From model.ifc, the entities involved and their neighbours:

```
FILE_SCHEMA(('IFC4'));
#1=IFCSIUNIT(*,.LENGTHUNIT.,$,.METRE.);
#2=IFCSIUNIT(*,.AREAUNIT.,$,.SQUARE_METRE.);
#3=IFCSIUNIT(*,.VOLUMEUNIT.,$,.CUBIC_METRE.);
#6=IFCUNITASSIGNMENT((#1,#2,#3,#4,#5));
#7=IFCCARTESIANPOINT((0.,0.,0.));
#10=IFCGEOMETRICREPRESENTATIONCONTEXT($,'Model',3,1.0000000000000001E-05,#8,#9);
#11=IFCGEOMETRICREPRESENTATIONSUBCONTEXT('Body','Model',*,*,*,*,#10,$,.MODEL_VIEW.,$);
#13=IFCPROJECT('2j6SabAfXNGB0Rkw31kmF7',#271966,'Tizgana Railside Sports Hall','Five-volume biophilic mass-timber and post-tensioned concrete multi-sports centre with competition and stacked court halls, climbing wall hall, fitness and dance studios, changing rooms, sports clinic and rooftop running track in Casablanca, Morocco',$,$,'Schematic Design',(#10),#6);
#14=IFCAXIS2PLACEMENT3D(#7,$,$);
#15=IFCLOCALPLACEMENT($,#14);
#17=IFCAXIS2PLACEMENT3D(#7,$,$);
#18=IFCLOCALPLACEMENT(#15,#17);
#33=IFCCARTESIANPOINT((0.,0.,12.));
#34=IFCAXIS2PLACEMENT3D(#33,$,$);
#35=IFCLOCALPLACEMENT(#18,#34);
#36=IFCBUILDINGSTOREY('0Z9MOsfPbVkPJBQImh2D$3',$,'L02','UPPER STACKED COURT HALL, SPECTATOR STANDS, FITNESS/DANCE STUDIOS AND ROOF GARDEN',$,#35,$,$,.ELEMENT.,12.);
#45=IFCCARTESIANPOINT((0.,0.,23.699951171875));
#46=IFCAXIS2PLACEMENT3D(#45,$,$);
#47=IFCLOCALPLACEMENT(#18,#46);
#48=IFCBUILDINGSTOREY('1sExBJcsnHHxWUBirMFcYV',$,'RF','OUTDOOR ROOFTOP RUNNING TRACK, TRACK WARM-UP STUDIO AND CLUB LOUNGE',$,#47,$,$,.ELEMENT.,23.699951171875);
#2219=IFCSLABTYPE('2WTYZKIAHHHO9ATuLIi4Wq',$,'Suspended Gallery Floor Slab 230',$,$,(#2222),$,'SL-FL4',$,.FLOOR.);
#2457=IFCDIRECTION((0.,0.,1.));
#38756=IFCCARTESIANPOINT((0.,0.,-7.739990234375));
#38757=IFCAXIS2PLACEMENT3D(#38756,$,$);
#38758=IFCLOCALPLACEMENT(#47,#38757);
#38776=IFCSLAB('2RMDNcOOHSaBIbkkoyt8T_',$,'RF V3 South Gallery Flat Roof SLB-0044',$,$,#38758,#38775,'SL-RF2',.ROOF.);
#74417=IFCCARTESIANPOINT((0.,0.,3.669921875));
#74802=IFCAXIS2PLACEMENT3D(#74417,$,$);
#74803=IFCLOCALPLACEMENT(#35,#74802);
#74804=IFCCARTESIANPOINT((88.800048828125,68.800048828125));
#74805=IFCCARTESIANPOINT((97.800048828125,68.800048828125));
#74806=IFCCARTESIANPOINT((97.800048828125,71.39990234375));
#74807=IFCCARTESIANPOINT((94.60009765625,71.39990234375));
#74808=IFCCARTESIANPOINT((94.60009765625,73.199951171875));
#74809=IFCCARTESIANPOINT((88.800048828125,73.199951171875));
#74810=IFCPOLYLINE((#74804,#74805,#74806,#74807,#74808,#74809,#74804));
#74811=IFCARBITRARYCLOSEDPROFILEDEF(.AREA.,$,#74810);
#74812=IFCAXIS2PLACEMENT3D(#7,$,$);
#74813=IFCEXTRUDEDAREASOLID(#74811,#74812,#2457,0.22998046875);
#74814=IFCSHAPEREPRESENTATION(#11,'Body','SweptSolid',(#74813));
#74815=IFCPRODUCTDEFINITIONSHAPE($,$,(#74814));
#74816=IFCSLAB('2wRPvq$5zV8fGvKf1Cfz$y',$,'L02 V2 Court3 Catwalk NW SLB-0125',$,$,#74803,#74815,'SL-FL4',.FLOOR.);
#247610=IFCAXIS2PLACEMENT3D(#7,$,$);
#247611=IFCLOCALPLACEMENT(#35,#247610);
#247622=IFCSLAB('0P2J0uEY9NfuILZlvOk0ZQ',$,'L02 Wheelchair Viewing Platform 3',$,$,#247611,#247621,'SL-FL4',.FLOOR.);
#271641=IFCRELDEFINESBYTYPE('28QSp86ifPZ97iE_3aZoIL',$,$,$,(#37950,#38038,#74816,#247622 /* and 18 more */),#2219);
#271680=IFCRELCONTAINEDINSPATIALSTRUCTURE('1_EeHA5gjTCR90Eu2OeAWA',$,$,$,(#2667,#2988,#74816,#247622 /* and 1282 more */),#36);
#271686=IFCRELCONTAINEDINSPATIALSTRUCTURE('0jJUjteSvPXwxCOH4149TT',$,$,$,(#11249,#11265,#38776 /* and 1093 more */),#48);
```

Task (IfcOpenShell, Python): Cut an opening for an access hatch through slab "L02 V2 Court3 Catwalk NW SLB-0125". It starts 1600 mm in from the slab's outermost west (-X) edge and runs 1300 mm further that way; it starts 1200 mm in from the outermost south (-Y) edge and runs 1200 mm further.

```python
import numpy as np
import ifcopenshell
import ifcopenshell.api.feature
import ifcopenshell.api.geometry
import ifcopenshell.api.root
import ifcopenshell.geom
import ifcopenshell.util.placement
import ifcopenshell.util.representation
import ifcopenshell.util.shape
import ifcopenshell.util.unit

model = ifcopenshell.open("model.ifc")
unit_scale = ifcopenshell.util.unit.calculate_unit_scale(model)
settings = ifcopenshell.geom.settings()


def volume(element):
    """Net volume in cubic metres, openings subtracted."""
    shape = ifcopenshell.geom.create_shape(settings, element)
    return ifcopenshell.util.shape.get_volume(shape.geometry)


slab = model.by_id(74816)
before = volume(slab)

# Extent in the slab's own axes, in metres. The edges named are its -X and -Y sides.
slab_shape = ifcopenshell.geom.create_shape(settings, slab)
vertices = ifcopenshell.util.shape.get_vertices(slab_shape.geometry)
x_min, y_min, bottom = vertices.min(axis=0)
top = vertices[:, 2].max()

opening = ifcopenshell.api.root.create_entity(model, ifc_class="IfcOpeningElement", name="Access hatch opening", predefined_type="OPENING")
context = ifcopenshell.util.representation.get_context(model, "Model", "Body", "MODEL_VIEW")
width, depth = 1.3, 1.2
outline = [(0.0, 0.0), (width, 0.0), (width, depth), (0.0, depth), (0.0, 0.0)]
# Overshoot both faces by 50 mm so the cut is clean.
shape = ifcopenshell.api.geometry.add_slab_representation(
    model, context=context, depth=top - bottom + 0.1, polyline=outline
)
ifcopenshell.api.geometry.assign_representation(model, product=opening, representation=shape)

matrix = ifcopenshell.util.placement.get_local_placement(slab.ObjectPlacement)
matrix[:, 3] = matrix @ np.append(np.array([x_min + 1.6, y_min + 1.2, bottom - 0.05]) / unit_scale, 1.0)
ifcopenshell.api.geometry.edit_object_placement(model, product=opening, matrix=matrix, is_si=False)
ifcopenshell.api.feature.add_feature(model, feature=opening, element=slab)

after = volume(slab)

print(f"slab volume {before:.3f} -> {after:.3f} m3")

model.write("model_v2.ifc")
```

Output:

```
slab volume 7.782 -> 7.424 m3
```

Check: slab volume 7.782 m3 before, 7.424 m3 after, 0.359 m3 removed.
